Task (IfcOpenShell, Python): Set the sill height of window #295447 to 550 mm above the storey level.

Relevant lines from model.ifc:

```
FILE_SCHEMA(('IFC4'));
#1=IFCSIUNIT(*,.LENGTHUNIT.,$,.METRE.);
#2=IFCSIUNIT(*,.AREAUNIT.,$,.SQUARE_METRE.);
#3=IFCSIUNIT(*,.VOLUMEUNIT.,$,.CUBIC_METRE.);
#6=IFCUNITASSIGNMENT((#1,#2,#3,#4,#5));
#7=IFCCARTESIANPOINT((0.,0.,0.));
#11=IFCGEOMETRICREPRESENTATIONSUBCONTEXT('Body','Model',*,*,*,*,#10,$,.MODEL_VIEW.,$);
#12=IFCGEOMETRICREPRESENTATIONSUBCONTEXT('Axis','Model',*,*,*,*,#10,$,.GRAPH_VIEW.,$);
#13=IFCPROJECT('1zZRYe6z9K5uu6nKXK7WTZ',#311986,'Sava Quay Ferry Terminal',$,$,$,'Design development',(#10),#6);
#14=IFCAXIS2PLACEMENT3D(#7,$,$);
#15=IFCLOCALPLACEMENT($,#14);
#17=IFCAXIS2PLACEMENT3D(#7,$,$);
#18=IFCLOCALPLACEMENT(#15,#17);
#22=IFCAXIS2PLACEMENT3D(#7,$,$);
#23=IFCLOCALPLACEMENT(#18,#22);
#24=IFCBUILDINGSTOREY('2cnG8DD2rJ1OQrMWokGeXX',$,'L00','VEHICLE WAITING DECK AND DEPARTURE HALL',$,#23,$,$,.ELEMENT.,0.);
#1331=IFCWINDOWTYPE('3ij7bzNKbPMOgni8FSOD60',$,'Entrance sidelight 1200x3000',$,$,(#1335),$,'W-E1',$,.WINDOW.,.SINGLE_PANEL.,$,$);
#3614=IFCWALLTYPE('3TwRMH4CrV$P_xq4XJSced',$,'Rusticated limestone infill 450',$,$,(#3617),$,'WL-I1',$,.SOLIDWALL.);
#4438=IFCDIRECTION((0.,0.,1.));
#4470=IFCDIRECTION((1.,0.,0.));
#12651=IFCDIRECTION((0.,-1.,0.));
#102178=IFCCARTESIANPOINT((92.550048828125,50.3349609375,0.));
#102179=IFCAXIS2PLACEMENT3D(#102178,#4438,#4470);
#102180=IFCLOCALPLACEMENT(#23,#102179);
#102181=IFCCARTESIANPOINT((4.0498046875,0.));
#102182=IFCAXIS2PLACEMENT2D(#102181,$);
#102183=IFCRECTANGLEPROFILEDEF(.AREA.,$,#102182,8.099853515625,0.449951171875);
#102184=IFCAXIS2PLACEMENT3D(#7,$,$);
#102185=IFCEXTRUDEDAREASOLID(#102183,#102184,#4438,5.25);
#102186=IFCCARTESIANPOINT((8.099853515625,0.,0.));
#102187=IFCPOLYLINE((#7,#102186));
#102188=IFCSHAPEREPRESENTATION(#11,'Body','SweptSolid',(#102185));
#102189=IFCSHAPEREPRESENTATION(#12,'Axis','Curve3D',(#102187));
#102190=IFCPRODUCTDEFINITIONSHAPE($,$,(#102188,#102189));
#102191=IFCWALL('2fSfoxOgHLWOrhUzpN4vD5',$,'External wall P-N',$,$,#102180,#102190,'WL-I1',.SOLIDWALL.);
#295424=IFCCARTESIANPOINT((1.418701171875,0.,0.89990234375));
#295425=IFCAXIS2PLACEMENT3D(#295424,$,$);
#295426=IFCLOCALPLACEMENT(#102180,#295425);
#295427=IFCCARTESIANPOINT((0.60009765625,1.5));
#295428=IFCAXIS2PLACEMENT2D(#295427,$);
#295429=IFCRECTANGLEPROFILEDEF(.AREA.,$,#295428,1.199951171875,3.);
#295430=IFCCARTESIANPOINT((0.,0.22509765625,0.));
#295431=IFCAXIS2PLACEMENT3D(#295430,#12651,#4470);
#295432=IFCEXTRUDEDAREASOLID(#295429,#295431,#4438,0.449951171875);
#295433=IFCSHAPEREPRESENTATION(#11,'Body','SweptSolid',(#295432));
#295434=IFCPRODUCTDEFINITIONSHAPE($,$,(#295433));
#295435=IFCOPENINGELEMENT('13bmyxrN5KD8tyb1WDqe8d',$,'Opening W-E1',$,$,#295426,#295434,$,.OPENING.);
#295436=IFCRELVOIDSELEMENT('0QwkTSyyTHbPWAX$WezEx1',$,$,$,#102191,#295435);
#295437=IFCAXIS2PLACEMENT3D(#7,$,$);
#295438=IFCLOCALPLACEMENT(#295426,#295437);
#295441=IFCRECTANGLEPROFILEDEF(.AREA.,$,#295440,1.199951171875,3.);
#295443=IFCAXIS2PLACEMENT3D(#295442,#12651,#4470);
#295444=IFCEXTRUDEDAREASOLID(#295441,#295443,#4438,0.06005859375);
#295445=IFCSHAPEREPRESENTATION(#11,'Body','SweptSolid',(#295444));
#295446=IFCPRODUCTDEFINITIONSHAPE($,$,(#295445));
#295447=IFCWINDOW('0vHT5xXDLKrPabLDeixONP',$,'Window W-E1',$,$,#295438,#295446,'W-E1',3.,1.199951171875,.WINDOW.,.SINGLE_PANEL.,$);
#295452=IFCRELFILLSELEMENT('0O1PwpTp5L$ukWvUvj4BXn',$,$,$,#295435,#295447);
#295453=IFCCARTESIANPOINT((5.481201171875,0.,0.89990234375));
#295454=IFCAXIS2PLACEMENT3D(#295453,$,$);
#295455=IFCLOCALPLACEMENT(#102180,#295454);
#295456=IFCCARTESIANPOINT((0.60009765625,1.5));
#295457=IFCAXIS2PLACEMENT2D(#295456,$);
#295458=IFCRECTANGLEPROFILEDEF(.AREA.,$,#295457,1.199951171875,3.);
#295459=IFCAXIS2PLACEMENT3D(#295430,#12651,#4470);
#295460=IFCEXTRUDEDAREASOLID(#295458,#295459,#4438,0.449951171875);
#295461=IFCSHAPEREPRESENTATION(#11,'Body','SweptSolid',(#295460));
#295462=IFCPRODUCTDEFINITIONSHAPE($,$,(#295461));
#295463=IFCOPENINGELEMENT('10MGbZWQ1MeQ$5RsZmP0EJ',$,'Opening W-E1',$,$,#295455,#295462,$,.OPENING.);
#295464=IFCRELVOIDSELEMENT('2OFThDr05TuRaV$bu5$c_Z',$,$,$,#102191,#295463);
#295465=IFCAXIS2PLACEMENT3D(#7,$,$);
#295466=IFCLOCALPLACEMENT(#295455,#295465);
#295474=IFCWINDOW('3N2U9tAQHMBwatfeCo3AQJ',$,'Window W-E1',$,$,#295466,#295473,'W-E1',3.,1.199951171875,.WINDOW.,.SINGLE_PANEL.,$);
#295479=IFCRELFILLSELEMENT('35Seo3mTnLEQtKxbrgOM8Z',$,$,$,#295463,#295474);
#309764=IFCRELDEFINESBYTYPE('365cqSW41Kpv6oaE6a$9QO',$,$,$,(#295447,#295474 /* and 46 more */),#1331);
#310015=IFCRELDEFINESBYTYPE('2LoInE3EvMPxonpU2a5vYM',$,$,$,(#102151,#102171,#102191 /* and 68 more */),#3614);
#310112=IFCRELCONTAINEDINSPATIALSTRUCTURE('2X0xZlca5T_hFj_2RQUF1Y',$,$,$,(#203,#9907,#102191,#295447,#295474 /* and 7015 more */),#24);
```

```python
import numpy as np
import ifcopenshell
import ifcopenshell.api.geometry
import ifcopenshell.geom
import ifcopenshell.util.element
import ifcopenshell.util.placement
import ifcopenshell.util.shape
import ifcopenshell.util.unit

model = ifcopenshell.open("model.ifc")
unit_scale = ifcopenshell.util.unit.calculate_unit_scale(model)

window = model.by_guid("0vHT5xXDLKrPabLDeixONP")
opening = window.FillsVoids[0].RelatingOpeningElement
storey = ifcopenshell.util.element.get_container(window, ifc_class="IfcBuildingStorey")
level = ifcopenshell.util.placement.get_local_placement(storey.ObjectPlacement)[2, 3]

# The opening's origin need not be at the sill, so measure its lowest point.
shape = ifcopenshell.geom.create_shape(ifcopenshell.geom.settings(), opening)
bottom = ifcopenshell.util.shape.get_shape_bottom_elevation(shape, shape.geometry) / unit_scale
dz = level + 0.55 - bottom

shift = np.array([0.0, 0.0, dz])
# The window is placed relative to its opening, so it follows when the opening moves.
matrix = ifcopenshell.util.placement.get_local_placement(opening.ObjectPlacement)
matrix[:3, 3] += shift
ifcopenshell.api.geometry.edit_object_placement(
    model, product=opening, matrix=matrix, is_si=False, should_transform_children=True
)

print(f"moved by {dz * unit_scale:+.3f} m")

model.write("model-out.ifc")
```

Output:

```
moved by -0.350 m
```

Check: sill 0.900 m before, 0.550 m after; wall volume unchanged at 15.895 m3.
